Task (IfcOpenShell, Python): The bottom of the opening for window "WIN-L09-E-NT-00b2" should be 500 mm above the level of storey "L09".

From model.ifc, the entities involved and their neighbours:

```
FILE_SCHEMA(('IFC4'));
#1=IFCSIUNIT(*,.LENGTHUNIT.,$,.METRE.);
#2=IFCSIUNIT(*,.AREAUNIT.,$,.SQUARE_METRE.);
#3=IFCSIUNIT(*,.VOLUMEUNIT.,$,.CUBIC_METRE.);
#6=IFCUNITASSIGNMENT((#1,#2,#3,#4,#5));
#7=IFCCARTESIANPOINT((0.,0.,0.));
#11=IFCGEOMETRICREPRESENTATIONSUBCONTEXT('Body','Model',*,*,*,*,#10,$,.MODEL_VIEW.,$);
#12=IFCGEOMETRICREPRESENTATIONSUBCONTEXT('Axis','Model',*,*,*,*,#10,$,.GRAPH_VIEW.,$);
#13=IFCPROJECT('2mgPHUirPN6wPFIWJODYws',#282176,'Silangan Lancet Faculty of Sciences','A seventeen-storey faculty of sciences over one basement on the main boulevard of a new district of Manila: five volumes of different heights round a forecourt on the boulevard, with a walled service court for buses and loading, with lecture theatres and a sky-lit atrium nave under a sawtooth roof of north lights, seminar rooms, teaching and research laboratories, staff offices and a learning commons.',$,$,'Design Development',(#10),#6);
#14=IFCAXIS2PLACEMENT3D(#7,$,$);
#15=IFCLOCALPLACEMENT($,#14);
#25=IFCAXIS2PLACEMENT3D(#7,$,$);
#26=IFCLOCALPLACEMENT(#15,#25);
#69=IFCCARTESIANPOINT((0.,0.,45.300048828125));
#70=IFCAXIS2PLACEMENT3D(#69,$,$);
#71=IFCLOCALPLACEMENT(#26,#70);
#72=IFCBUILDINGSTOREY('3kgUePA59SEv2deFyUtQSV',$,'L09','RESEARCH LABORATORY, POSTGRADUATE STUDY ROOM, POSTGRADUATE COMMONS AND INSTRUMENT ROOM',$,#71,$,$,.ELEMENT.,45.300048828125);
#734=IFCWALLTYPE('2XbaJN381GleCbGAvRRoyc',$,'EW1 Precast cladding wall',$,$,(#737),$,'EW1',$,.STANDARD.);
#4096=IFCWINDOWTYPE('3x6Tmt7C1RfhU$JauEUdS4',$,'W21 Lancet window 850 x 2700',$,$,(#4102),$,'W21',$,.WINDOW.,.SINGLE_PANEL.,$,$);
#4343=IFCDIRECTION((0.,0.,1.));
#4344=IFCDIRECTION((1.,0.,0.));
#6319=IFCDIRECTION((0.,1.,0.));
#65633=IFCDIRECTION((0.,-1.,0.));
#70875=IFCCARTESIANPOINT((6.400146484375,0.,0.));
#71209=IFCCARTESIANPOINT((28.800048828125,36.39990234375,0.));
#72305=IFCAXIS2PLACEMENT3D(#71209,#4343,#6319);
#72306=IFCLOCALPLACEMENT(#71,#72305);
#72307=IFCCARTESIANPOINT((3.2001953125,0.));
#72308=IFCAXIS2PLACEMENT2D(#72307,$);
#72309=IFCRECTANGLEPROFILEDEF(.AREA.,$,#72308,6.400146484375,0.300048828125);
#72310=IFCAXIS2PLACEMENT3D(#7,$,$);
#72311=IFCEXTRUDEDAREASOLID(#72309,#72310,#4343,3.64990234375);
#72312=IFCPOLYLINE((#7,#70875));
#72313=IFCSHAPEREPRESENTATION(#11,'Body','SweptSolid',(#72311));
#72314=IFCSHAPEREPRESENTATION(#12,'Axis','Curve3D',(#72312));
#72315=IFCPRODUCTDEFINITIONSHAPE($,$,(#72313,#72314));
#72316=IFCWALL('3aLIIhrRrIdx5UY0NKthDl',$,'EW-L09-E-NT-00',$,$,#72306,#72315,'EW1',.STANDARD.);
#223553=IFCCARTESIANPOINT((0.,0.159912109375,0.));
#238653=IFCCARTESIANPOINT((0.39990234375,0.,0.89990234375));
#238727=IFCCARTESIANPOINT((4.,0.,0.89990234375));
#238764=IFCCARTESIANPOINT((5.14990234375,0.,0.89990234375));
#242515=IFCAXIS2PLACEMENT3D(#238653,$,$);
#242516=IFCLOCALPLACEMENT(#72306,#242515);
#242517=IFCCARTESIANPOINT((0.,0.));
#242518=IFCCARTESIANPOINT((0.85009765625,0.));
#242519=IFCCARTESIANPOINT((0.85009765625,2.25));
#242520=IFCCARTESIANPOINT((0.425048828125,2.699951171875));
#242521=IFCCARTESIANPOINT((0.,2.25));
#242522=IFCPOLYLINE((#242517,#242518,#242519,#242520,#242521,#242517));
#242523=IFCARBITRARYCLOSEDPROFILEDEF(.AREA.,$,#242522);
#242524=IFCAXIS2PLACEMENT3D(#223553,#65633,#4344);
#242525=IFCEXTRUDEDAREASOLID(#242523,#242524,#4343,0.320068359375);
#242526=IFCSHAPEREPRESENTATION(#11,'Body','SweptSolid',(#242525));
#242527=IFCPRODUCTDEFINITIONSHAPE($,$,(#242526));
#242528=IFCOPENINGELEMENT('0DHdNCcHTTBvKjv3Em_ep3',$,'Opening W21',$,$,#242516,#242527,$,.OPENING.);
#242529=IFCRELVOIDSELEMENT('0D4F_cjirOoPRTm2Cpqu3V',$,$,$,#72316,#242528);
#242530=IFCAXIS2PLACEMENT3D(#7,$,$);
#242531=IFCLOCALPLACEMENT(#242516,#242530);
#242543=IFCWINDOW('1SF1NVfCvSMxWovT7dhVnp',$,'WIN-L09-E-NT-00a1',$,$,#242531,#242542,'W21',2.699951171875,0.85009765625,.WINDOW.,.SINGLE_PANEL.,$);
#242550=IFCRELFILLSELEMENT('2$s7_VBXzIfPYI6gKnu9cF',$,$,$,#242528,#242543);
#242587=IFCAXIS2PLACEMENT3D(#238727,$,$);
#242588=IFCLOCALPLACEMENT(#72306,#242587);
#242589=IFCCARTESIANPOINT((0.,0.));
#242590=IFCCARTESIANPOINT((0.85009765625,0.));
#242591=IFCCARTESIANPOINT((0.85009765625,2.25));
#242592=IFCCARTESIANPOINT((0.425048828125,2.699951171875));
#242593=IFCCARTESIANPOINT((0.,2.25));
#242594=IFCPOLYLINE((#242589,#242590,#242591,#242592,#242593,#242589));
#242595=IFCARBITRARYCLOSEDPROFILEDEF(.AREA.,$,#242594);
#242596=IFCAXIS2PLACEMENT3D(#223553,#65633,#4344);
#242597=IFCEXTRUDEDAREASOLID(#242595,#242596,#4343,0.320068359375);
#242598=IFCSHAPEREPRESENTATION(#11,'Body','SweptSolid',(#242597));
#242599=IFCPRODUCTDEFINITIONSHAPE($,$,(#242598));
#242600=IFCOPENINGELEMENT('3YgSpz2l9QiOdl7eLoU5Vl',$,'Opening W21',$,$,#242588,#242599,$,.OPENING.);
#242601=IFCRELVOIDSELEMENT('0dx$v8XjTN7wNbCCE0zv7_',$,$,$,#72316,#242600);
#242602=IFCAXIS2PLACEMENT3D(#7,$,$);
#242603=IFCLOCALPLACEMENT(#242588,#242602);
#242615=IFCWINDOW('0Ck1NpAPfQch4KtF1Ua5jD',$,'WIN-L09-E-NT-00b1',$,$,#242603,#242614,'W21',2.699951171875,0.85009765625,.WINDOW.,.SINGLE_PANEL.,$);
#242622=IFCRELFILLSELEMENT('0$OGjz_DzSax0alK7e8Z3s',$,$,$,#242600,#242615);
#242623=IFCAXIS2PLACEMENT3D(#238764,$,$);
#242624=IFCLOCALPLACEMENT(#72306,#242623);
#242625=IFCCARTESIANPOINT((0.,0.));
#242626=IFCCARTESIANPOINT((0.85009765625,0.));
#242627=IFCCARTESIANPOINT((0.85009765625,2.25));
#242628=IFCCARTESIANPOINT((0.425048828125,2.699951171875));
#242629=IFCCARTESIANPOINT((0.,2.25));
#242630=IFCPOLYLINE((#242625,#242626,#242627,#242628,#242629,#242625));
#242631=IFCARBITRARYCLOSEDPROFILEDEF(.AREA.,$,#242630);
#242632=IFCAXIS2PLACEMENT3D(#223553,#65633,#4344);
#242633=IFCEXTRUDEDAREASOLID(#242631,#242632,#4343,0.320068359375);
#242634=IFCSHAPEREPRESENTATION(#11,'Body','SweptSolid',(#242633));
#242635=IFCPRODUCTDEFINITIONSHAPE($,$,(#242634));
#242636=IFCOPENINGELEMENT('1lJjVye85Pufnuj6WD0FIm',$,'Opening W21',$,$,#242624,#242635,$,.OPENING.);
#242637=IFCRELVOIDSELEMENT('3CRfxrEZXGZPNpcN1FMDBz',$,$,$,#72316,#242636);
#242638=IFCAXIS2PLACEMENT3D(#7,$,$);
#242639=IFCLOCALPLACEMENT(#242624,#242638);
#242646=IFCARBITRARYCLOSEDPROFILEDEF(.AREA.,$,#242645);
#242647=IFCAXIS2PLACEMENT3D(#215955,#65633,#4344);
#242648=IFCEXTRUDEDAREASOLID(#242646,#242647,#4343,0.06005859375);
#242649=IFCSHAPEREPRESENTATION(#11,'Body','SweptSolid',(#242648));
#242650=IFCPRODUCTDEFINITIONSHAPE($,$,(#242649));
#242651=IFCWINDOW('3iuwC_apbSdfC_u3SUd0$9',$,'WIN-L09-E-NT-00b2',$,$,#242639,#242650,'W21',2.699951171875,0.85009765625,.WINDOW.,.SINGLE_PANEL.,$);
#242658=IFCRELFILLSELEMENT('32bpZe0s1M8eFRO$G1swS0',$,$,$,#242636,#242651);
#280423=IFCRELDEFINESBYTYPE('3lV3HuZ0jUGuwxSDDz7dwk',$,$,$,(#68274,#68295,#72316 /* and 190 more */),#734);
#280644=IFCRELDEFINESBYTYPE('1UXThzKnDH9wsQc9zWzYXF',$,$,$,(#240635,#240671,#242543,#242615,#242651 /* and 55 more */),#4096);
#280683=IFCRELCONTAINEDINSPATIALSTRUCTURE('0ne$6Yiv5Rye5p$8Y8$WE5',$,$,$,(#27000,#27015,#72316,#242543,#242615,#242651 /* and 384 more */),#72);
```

```python
import numpy as np
import ifcopenshell
import ifcopenshell.api.geometry
import ifcopenshell.geom
import ifcopenshell.util.element
import ifcopenshell.util.placement
import ifcopenshell.util.shape
import ifcopenshell.util.unit

model = ifcopenshell.open("model.ifc")
unit_scale = ifcopenshell.util.unit.calculate_unit_scale(model)

window = model.by_guid("3iuwC_apbSdfC_u3SUd0$9")
opening = window.FillsVoids[0].RelatingOpeningElement
storey = ifcopenshell.util.element.get_container(window, ifc_class="IfcBuildingStorey")
level = ifcopenshell.util.placement.get_local_placement(storey.ObjectPlacement)[2, 3]

# The opening's origin need not be at the sill, so measure its lowest point.
shape = ifcopenshell.geom.create_shape(ifcopenshell.geom.settings(), opening)
bottom = ifcopenshell.util.shape.get_shape_bottom_elevation(shape, shape.geometry) / unit_scale
dz = level + 0.5 / unit_scale - bottom

shift = np.array([0.0, 0.0, dz])
# The window is placed relative to its opening, so it follows when the opening moves.
matrix = ifcopenshell.util.placement.get_local_placement(opening.ObjectPlacement)
matrix[:3, 3] += shift
ifcopenshell.api.geometry.edit_object_placement(
    model, product=opening, matrix=matrix, is_si=False, should_transform_children=True
)

print(f"moved by {dz * unit_scale:+.3f} m")

model.write("model_updated.ifc")
```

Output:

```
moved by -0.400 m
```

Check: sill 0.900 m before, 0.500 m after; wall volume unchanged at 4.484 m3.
